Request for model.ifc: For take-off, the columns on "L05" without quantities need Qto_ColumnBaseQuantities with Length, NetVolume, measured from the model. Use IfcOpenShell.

First a look at what the model holds.

```python
import ifcopenshell
import ifcopenshell.util.element
import ifcopenshell.util.unit

model = ifcopenshell.open("model.ifc")
print(model.schema)
for unit_type in ("LENGTHUNIT", "AREAUNIT", "VOLUMEUNIT"):
    print(unit_type, ifcopenshell.util.unit.calculate_unit_scale(model, unit_type))
storey = next(s for s in model.by_type("IfcBuildingStorey") if s.Name == "L05")
columns = [e for e in ifcopenshell.util.element.get_decomposition(storey) if e.is_a("IfcColumn")]
for e in sorted(columns, key=lambda e: e.id()):
    print(e.id(), e.is_a(), e.Name, list(ifcopenshell.util.element.get_psets(e, qtos_only=True)), sep=" | ")
```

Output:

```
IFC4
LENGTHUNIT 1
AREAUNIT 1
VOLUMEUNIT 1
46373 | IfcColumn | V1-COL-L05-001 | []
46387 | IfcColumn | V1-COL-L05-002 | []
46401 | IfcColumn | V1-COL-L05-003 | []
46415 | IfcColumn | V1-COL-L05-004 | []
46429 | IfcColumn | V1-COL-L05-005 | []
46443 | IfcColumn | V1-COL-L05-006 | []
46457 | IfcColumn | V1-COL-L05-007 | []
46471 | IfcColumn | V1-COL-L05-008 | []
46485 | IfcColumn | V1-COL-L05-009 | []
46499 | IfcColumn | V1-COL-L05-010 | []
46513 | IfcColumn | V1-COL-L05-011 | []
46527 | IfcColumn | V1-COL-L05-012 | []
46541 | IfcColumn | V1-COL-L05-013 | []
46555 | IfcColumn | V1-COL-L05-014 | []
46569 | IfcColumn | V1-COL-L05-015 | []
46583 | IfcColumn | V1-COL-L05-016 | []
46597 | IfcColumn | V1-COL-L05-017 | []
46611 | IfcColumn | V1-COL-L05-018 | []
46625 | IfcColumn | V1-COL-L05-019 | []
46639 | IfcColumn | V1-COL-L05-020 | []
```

```python
import ifcopenshell
import ifcopenshell.api.pset
import ifcopenshell.geom
import ifcopenshell.util.element
import ifcopenshell.util.shape
import ifcopenshell.util.unit

model = ifcopenshell.open("model.ifc")
unit_scale = ifcopenshell.util.unit.calculate_unit_scale(model)
volume_scale = ifcopenshell.util.unit.calculate_unit_scale(model, "VOLUMEUNIT")
settings = ifcopenshell.geom.settings()

storey = next(s for s in model.by_type("IfcBuildingStorey") if s.Name == "L05")
columns = [e for e in ifcopenshell.util.element.get_decomposition(storey) if e.is_a("IfcColumn")]

for e in sorted(columns, key=lambda e: e.id()):
    if ifcopenshell.util.element.get_psets(e, qtos_only=True, should_inherit=False):
        continue
    # Geometry comes back in metres, in the element's own axes.
    shape = ifcopenshell.geom.create_shape(settings, e)
    values = {
        "Length": ifcopenshell.util.shape.get_z(shape.geometry) / unit_scale,
        "NetVolume": ifcopenshell.util.shape.get_volume(shape.geometry) / volume_scale,
    }
    qto = ifcopenshell.api.pset.add_qto(model, product=e, name="Qto_ColumnBaseQuantities")
    ifcopenshell.api.pset.edit_qto(model, qto=qto, properties=values)
    print(e.id(), {k: round(v, 3) for k, v in values.items()})

model.write("model_updated.ifc")
```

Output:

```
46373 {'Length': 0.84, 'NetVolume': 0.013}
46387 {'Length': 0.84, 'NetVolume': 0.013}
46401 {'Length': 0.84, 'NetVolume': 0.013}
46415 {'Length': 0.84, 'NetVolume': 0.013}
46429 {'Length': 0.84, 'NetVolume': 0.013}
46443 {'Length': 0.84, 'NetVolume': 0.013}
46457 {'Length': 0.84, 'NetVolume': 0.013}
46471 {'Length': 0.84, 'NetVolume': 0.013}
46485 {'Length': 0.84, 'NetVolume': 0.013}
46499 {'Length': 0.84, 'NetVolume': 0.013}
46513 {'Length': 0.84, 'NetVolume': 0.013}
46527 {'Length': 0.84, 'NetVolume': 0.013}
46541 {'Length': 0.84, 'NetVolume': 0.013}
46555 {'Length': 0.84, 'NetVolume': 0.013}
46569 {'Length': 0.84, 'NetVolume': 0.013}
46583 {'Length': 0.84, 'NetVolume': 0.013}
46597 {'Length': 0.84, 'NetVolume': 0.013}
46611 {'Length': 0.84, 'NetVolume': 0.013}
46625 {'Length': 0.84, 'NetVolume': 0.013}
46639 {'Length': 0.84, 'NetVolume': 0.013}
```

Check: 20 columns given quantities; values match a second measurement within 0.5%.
